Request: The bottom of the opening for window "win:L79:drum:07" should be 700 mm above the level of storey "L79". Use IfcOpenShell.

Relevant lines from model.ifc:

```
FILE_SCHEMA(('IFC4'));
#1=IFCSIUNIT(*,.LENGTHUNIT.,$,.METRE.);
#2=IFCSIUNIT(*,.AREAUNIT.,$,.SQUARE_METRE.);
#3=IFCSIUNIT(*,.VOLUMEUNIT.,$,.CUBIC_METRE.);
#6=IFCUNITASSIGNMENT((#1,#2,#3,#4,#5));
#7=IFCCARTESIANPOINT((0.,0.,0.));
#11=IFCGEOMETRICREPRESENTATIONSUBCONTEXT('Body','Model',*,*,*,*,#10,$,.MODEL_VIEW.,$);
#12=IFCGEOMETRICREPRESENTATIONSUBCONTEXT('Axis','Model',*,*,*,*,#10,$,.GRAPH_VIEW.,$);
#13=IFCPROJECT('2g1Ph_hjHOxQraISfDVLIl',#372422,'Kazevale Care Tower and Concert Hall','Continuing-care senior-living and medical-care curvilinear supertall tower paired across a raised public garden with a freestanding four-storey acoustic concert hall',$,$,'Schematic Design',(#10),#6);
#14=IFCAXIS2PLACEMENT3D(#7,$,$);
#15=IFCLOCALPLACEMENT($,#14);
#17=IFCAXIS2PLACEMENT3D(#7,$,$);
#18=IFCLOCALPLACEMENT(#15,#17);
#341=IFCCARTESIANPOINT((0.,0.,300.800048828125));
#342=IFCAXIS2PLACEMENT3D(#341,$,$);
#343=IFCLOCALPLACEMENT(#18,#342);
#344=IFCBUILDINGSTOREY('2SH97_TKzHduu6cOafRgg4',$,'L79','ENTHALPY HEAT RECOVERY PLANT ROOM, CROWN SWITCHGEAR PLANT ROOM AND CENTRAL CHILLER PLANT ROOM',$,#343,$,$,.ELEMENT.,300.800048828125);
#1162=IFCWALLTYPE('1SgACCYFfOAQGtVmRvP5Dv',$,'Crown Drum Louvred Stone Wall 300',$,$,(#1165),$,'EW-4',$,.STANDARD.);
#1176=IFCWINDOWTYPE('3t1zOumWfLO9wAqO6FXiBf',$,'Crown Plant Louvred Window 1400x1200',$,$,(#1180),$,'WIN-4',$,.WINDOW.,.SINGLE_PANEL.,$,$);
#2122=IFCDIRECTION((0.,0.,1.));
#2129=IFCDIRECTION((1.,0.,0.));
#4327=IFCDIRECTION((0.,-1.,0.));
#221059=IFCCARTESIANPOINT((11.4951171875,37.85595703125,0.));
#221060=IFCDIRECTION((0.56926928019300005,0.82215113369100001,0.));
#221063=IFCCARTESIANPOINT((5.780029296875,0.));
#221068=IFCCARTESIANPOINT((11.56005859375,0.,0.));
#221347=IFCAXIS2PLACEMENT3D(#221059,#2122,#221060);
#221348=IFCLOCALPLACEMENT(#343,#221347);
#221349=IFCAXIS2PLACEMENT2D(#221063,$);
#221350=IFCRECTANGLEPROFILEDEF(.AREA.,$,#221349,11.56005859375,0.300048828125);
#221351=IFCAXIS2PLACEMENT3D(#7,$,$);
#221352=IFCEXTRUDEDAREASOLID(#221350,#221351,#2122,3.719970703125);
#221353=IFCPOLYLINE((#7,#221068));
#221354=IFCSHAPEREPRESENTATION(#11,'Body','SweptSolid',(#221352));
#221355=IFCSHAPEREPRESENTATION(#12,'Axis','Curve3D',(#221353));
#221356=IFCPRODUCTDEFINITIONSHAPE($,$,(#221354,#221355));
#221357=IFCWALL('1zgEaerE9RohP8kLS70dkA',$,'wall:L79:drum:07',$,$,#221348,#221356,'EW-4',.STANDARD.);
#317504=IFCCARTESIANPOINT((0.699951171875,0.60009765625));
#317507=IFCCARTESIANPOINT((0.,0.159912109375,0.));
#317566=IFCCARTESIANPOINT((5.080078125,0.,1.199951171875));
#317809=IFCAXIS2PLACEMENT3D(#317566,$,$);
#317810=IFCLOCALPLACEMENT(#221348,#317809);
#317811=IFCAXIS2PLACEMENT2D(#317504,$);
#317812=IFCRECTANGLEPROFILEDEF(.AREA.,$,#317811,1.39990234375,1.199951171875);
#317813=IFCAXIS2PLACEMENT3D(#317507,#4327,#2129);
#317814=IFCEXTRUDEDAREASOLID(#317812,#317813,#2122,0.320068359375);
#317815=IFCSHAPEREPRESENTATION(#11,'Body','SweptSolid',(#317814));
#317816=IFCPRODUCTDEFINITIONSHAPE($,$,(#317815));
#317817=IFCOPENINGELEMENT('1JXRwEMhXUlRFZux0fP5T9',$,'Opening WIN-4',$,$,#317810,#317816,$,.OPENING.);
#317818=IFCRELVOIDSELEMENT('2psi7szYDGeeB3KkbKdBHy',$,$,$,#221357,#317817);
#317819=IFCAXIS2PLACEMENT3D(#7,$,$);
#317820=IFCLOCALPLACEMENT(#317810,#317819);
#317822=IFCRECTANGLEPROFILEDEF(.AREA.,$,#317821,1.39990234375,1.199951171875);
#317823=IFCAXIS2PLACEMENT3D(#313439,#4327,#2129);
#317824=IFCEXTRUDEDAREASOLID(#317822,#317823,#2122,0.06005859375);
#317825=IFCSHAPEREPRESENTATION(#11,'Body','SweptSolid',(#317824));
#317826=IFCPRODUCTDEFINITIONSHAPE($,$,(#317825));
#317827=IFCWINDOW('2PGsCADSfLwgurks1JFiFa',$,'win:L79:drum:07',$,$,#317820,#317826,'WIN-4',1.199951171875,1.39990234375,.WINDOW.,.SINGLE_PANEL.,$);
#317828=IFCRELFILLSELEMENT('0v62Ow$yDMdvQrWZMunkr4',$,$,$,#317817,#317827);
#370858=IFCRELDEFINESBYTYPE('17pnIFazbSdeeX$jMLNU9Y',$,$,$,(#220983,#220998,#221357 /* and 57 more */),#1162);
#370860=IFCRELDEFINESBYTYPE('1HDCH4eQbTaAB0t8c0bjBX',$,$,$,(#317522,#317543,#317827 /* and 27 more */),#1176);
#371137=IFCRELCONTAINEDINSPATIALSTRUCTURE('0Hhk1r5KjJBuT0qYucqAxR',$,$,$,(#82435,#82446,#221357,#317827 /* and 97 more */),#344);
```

```python
import numpy as np
import ifcopenshell
import ifcopenshell.api.geometry
import ifcopenshell.geom
import ifcopenshell.util.element
import ifcopenshell.util.placement
import ifcopenshell.util.shape
import ifcopenshell.util.unit

model = ifcopenshell.open("model.ifc")
unit_scale = ifcopenshell.util.unit.calculate_unit_scale(model)

window = model.by_guid("2PGsCADSfLwgurks1JFiFa")
opening = window.FillsVoids[0].RelatingOpeningElement
storey = ifcopenshell.util.element.get_container(window, ifc_class="IfcBuildingStorey")
level = ifcopenshell.util.placement.get_local_placement(storey.ObjectPlacement)[2, 3]

# The opening's origin need not be at the sill, so measure its lowest point.
shape = ifcopenshell.geom.create_shape(ifcopenshell.geom.settings(), opening)
bottom = ifcopenshell.util.shape.get_shape_bottom_elevation(shape, shape.geometry) / unit_scale
dz = level + 0.7 - bottom

shift = np.array([0.0, 0.0, dz])
# The window is placed relative to its opening, so it follows when the opening moves.
matrix = ifcopenshell.util.placement.get_local_placement(opening.ObjectPlacement)
matrix[:3, 3] += shift
ifcopenshell.api.geometry.edit_object_placement(
    model, product=opening, matrix=matrix, is_si=False, should_transform_children=True
)

print(f"moved by {dz * unit_scale:+.3f} m")

model.write("model_rev.ifc")
```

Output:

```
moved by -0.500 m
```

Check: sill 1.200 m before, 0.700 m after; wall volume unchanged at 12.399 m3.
